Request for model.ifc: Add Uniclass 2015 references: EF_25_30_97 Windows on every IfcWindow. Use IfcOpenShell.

First a look at what the model holds.

```python
import ifcopenshell

model = ifcopenshell.open("model.ifc")
print(model.schema)
print("classifications:", [c.Name for c in model.by_type("IfcClassification")])
for ifc_class in ("IfcDoor", "IfcRoof", "IfcStair", "IfcWall", "IfcWindow"):
    print(ifc_class, len(model.by_type(ifc_class)))
```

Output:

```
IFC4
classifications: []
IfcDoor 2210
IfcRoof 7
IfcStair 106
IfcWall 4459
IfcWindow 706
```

```python
import ifcopenshell
import ifcopenshell.api.classification

model = ifcopenshell.open("model.ifc")

system = ifcopenshell.api.classification.add_classification(model, classification="Uniclass 2015")

codes = {
    "IfcWindow": ("EF_25_30_97", "Windows"),
}
for ifc_class, (code, name) in codes.items():
    products = model.by_type(ifc_class)
    ifcopenshell.api.classification.add_reference(
        model, products=products, classification=system, identification=code, name=name
    )
    print(code, len(products))

model.write("model-out.ifc")
```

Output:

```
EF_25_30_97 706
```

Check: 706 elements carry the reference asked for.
